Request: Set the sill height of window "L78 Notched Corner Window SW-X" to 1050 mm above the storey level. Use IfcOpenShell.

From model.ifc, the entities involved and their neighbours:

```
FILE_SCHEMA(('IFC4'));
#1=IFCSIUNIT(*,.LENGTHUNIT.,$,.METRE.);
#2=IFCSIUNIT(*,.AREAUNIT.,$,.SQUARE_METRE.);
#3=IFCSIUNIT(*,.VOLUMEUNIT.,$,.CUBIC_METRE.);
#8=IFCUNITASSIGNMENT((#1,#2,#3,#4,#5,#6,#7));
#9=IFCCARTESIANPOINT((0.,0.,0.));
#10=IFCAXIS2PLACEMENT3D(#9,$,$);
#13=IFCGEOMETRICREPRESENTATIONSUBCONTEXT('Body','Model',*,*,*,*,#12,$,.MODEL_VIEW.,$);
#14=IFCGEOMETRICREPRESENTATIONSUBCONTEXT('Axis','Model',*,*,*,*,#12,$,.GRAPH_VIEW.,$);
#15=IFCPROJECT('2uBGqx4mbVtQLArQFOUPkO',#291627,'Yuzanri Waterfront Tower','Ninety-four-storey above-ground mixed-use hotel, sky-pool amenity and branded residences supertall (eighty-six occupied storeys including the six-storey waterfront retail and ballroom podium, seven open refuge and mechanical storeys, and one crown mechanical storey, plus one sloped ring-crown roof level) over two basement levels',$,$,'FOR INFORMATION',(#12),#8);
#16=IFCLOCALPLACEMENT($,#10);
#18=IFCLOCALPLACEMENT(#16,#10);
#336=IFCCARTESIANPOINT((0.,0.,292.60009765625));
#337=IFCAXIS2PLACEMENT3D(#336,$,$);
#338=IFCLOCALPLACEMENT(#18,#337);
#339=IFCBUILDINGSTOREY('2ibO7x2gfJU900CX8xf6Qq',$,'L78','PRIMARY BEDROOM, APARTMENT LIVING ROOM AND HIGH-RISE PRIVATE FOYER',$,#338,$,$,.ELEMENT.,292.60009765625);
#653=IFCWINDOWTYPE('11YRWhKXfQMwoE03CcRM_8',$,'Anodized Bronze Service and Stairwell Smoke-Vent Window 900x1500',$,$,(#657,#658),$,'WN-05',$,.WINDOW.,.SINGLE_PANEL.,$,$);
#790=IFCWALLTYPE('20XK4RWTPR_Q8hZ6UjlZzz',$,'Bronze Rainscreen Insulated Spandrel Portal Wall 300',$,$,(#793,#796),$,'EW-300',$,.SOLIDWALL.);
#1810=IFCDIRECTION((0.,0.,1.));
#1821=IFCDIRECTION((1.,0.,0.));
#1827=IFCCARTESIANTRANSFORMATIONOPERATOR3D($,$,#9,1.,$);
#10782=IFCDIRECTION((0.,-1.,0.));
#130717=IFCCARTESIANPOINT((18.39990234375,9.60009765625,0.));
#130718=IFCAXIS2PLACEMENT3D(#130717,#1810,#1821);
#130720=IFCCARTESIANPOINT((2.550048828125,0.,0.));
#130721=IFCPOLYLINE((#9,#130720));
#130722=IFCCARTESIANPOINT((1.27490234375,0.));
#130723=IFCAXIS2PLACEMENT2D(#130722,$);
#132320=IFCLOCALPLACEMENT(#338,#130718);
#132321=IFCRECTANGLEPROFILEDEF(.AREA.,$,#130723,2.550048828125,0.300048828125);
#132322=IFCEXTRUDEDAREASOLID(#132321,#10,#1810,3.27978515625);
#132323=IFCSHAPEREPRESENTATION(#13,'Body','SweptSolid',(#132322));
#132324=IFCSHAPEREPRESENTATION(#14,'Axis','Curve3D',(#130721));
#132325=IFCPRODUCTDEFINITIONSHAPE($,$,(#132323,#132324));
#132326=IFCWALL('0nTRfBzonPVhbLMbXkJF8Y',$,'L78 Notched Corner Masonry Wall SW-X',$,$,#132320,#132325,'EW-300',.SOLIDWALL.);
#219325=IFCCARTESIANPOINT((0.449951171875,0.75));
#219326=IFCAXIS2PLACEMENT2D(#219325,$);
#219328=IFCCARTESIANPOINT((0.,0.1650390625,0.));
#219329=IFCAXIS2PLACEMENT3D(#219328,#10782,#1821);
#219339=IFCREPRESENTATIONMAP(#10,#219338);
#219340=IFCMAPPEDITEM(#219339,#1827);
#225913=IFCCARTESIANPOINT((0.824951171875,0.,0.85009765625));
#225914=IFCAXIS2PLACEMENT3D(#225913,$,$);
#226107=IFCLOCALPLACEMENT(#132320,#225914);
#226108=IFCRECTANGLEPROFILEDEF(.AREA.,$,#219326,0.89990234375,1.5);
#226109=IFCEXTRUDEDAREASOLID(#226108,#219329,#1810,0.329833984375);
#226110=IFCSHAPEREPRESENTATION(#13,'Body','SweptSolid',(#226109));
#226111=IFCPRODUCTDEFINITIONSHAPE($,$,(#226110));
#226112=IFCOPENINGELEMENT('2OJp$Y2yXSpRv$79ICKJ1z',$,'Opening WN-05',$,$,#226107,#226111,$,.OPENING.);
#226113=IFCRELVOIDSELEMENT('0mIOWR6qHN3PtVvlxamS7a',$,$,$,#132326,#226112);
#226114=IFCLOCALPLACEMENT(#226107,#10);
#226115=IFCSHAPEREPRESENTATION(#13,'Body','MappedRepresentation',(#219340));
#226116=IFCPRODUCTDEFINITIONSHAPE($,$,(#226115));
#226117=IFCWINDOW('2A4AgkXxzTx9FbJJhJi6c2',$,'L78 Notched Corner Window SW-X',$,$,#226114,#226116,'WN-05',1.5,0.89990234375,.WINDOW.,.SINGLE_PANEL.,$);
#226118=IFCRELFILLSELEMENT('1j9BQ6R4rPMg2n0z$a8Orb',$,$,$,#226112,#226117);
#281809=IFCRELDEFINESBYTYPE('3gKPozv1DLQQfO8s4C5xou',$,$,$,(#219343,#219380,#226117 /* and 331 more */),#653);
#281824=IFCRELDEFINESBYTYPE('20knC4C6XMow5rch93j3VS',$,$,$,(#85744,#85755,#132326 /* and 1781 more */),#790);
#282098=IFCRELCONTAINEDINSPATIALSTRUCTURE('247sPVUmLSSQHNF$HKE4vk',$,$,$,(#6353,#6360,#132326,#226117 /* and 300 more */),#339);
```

```python
import numpy as np
import ifcopenshell
import ifcopenshell.api.geometry
import ifcopenshell.geom
import ifcopenshell.util.element
import ifcopenshell.util.placement
import ifcopenshell.util.shape
import ifcopenshell.util.unit

model = ifcopenshell.open("model.ifc")
unit_scale = ifcopenshell.util.unit.calculate_unit_scale(model)

window = model.by_id(226117)
opening = window.FillsVoids[0].RelatingOpeningElement
storey = ifcopenshell.util.element.get_container(window, ifc_class="IfcBuildingStorey")
level = ifcopenshell.util.placement.get_local_placement(storey.ObjectPlacement)[2, 3]

# The opening's origin need not be at the sill, so measure its lowest point.
shape = ifcopenshell.geom.create_shape(ifcopenshell.geom.settings(), opening)
bottom = ifcopenshell.util.shape.get_shape_bottom_elevation(shape, shape.geometry) / unit_scale
dz = level + 1.05 / unit_scale - bottom

shift = np.array([0.0, 0.0, dz])
# The window is placed relative to its opening, so it follows when the opening moves.
matrix = ifcopenshell.util.placement.get_local_placement(opening.ObjectPlacement)
matrix[:3, 3] += shift
ifcopenshell.api.geometry.edit_object_placement(
    model, product=opening, matrix=matrix, is_si=False, should_transform_children=True
)

print(f"moved by {dz * unit_scale:+.3f} m")

model.write("model_edited.ifc")
```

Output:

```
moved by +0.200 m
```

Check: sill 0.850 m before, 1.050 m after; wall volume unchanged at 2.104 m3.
